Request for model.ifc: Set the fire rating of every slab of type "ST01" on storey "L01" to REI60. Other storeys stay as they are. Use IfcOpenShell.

First a look at what the model holds.

```python
import ifcopenshell
import ifcopenshell.util.element

model = ifcopenshell.open("model.ifc")
print(model.schema)
storey = next(s for s in model.by_type("IfcBuildingStorey") if s.Name == "L01")
slabs = [e for e in ifcopenshell.util.element.get_decomposition(storey) if e.is_a("IfcSlab")]
seen = {}
for e in slabs:
    element_type = ifcopenshell.util.element.get_type(e)
    key = (element_type.Name if element_type != e and element_type else None, ifcopenshell.util.element.get_pset(e, "Pset_SlabCommon", "FireRating"))
    seen[key] = seen.get(key, 0) + 1
for (name, value), count in sorted(seen.items(), key=str):
    print(count, "x", name, "|", value)
```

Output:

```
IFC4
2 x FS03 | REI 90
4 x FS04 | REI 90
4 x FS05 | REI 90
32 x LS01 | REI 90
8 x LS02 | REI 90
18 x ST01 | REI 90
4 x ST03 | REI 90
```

```python
import ifcopenshell
import ifcopenshell.api.pset
import ifcopenshell.util.element

model = ifcopenshell.open("model.ifc")

storey = next(s for s in model.by_type("IfcBuildingStorey") if s.Name == "L01")
slabs = [e for e in ifcopenshell.util.element.get_decomposition(storey) if e.is_a("IfcSlab")]

count = 0
for e in slabs:
    element_type = ifcopenshell.util.element.get_type(e)
    if element_type in (None, e) or element_type.Name != "ST01":
        continue
    # add_pset returns the element's existing set when there is one.
    pset = ifcopenshell.api.pset.add_pset(model, product=e, name="Pset_SlabCommon")
    ifcopenshell.api.pset.edit_pset(model, pset=pset, properties={"FireRating": "REI60"})
    count += 1

print(count, "slabs updated")

model.write("model_updated.ifc")
```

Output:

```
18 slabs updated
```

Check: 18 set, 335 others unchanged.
